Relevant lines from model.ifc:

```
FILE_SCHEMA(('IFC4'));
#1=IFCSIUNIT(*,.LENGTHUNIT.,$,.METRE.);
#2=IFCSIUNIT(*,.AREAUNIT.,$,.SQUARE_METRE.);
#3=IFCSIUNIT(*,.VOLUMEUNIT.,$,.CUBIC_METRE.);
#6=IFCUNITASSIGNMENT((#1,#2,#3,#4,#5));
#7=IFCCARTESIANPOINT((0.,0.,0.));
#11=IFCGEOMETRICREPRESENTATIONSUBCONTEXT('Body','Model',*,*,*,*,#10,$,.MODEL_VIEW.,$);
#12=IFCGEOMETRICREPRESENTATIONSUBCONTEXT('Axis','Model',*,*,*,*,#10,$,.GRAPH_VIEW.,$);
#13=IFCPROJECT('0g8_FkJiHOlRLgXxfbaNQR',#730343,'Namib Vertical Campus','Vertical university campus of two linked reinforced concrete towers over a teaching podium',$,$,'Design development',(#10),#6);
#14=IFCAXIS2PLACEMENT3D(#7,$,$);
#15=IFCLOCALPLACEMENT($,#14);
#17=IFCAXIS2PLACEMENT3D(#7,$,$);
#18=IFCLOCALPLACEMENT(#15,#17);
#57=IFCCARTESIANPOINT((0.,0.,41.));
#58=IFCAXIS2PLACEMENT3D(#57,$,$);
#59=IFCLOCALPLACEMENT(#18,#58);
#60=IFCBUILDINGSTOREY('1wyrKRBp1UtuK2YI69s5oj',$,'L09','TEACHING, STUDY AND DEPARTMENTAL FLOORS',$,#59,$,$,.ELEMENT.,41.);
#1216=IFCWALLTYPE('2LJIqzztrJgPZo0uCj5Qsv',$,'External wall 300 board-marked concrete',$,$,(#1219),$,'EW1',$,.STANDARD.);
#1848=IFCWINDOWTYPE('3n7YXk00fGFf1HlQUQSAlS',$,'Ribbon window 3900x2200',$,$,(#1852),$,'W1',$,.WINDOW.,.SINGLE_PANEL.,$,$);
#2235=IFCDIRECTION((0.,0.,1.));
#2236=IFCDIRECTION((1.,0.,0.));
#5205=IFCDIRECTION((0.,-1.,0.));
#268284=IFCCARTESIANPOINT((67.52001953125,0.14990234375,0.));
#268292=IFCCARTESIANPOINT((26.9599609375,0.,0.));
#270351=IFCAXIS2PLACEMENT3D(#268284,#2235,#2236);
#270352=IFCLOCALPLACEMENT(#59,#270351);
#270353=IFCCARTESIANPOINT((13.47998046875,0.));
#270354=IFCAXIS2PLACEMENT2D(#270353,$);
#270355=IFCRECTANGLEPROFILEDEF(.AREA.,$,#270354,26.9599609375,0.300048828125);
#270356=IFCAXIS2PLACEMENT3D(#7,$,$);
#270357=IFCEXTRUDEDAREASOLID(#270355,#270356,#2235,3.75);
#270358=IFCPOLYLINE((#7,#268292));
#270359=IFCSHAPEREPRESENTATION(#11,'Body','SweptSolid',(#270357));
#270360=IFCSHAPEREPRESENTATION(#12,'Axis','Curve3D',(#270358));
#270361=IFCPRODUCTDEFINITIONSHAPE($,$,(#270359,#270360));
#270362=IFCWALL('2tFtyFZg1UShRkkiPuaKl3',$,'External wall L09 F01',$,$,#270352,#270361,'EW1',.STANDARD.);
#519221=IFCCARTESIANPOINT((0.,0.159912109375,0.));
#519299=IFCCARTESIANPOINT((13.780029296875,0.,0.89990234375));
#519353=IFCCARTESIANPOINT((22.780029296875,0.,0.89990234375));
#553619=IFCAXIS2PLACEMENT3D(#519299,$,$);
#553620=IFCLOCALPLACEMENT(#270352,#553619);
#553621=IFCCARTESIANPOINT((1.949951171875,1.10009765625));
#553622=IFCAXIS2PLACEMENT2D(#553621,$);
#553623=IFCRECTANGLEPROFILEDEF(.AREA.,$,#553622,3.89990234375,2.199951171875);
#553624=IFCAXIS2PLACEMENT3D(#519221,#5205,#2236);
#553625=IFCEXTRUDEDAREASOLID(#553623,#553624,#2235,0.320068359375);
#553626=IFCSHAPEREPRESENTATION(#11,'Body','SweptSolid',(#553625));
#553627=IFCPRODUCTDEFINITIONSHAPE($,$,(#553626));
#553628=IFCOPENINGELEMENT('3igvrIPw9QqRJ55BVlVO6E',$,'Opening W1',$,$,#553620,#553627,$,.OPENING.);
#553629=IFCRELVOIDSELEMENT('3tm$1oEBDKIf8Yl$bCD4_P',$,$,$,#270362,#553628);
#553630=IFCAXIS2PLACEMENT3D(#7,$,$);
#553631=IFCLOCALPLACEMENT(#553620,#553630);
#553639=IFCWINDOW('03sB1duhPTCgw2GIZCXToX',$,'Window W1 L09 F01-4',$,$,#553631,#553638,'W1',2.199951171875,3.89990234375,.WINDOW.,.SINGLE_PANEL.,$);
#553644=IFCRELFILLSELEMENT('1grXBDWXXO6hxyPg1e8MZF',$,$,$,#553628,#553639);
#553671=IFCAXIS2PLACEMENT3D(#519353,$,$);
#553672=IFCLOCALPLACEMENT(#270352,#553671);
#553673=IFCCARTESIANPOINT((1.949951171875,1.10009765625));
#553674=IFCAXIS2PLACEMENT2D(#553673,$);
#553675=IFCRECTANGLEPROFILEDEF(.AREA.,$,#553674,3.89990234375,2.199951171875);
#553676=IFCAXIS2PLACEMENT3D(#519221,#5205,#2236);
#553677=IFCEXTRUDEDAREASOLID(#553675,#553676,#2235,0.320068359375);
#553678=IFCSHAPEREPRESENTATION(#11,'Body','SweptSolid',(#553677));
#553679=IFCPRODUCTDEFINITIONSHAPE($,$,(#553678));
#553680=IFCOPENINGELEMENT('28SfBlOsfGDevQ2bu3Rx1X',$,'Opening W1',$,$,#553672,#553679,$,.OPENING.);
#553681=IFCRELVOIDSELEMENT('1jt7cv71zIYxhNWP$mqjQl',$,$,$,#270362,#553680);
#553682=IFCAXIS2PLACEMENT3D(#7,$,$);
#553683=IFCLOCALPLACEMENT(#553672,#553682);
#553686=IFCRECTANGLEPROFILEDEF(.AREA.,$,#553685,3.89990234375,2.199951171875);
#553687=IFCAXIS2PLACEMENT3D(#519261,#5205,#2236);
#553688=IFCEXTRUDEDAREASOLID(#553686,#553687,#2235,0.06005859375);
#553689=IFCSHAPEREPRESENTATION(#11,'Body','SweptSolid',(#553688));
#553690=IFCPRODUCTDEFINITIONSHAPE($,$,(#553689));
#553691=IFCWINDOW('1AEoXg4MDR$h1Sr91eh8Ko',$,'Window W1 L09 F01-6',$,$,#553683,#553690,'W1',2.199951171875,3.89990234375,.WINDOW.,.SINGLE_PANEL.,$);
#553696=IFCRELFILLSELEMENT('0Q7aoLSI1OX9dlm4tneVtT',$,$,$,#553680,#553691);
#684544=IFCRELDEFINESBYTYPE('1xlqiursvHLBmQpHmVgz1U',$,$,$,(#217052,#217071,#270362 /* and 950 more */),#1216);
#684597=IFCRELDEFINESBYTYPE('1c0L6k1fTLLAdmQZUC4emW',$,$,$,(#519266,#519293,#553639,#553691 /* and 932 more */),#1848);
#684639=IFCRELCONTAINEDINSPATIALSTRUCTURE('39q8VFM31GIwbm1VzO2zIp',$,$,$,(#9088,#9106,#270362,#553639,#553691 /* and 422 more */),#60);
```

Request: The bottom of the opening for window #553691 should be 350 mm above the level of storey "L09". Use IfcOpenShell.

```python
import numpy as np
import ifcopenshell
import ifcopenshell.api.geometry
import ifcopenshell.geom
import ifcopenshell.util.element
import ifcopenshell.util.placement
import ifcopenshell.util.shape
import ifcopenshell.util.unit

model = ifcopenshell.open("model.ifc")
unit_scale = ifcopenshell.util.unit.calculate_unit_scale(model)

window = model.by_guid("1AEoXg4MDR$h1Sr91eh8Ko")
opening = window.FillsVoids[0].RelatingOpeningElement
storey = ifcopenshell.util.element.get_container(window, ifc_class="IfcBuildingStorey")
level = ifcopenshell.util.placement.get_local_placement(storey.ObjectPlacement)[2, 3]

# The opening's origin need not be at the sill, so measure its lowest point.
shape = ifcopenshell.geom.create_shape(ifcopenshell.geom.settings(), opening)
bottom = ifcopenshell.util.shape.get_shape_bottom_elevation(shape, shape.geometry) / unit_scale
dz = level + 0.35 - bottom

shift = np.array([0.0, 0.0, dz])
# The window is placed relative to its opening, so it follows when the opening moves.
matrix = ifcopenshell.util.placement.get_local_placement(opening.ObjectPlacement)
matrix[:3, 3] += shift
ifcopenshell.api.geometry.edit_object_placement(
    model, product=opening, matrix=matrix, is_si=False, should_transform_children=True
)

print(f"moved by {dz * unit_scale:+.3f} m")

model.write("model_v2.ifc")
```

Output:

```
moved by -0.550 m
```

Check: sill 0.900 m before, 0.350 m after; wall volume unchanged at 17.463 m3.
